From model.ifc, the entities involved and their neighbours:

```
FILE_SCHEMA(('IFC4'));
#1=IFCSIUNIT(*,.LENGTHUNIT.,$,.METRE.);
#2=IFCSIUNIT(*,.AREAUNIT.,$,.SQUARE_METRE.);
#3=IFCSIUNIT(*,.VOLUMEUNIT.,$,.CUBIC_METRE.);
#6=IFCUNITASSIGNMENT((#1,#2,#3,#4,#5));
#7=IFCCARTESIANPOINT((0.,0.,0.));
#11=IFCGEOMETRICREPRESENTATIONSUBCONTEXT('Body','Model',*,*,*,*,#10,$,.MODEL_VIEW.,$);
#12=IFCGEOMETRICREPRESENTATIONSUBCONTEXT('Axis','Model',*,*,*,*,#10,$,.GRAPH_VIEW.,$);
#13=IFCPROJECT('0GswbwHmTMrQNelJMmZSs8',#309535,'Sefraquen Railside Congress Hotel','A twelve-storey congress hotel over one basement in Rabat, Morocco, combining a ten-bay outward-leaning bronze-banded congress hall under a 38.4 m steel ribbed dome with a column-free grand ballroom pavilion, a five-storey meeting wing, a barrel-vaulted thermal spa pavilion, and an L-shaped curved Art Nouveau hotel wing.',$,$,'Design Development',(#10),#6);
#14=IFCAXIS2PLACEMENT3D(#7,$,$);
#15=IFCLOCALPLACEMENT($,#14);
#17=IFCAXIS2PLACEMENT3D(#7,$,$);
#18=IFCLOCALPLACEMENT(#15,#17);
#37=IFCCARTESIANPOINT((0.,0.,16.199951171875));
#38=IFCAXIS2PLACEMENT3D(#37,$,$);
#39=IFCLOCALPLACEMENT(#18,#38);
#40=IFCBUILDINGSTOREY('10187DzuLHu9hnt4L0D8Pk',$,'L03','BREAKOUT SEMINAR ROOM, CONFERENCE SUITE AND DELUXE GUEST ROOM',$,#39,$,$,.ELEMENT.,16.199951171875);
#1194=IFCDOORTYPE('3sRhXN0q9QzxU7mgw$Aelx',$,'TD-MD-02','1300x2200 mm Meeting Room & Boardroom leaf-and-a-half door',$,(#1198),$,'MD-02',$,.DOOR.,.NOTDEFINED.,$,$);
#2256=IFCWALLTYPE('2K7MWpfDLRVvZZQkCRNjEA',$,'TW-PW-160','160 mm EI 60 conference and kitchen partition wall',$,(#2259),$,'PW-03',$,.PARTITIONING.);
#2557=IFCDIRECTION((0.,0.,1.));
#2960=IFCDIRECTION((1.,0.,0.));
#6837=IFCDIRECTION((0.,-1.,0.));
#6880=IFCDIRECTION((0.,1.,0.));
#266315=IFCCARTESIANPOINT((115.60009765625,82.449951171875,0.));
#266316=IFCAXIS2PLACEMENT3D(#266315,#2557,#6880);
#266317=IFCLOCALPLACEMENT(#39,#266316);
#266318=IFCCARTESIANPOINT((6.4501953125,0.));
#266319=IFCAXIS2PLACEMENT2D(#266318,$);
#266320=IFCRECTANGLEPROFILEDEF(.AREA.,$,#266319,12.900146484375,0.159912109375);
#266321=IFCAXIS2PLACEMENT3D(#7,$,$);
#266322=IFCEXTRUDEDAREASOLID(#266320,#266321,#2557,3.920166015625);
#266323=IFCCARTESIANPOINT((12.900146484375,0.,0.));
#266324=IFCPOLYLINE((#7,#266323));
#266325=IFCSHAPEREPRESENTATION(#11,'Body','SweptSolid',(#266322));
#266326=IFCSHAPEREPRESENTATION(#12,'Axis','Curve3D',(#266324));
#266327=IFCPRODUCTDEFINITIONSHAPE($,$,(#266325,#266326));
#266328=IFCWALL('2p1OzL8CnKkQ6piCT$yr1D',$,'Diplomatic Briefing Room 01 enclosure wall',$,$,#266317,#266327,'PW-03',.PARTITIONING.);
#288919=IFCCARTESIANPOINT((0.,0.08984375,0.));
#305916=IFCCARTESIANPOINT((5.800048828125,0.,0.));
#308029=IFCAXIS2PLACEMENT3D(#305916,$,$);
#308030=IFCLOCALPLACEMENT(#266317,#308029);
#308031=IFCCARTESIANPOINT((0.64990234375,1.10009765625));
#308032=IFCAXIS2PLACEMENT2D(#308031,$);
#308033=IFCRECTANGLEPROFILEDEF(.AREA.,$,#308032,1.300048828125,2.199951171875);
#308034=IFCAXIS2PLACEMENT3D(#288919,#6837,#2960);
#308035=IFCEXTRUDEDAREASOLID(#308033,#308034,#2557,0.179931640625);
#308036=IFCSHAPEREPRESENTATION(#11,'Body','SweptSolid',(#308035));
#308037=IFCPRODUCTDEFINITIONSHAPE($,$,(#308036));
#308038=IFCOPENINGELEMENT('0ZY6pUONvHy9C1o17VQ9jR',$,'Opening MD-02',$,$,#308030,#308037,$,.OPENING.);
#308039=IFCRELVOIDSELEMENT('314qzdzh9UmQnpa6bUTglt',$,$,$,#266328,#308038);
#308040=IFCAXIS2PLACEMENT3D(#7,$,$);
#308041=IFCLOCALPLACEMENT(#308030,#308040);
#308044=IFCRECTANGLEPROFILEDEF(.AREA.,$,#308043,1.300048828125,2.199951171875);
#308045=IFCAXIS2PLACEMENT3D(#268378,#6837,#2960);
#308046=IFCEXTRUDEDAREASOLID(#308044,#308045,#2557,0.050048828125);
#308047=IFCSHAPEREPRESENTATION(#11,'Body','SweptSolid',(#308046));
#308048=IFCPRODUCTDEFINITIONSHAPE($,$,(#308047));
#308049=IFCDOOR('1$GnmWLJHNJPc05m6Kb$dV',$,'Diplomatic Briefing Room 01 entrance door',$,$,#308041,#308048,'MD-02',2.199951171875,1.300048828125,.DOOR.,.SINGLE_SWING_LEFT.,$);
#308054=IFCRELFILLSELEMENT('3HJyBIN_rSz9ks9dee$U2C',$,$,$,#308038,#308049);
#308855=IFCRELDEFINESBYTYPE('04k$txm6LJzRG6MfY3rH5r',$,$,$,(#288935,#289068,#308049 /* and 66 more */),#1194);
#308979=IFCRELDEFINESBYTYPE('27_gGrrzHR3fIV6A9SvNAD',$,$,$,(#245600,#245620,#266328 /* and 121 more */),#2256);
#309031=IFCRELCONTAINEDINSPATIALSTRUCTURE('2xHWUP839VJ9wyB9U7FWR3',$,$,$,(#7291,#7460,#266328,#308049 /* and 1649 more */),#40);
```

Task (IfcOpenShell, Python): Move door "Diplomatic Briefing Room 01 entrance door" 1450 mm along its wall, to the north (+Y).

```python
import ifcopenshell
import ifcopenshell.api.geometry
import ifcopenshell.util.placement
import ifcopenshell.util.unit

model = ifcopenshell.open("model.ifc")
unit_scale = ifcopenshell.util.unit.calculate_unit_scale(model)

door = model.by_id(308049)
opening = door.FillsVoids[0].RelatingOpeningElement
wall = opening.VoidsElements[0].RelatingBuildingElement

wall_matrix = ifcopenshell.util.placement.get_local_placement(wall.ObjectPlacement)
shift = wall_matrix[:3, 0] * 1.45 / unit_scale
before = ifcopenshell.util.placement.get_local_placement(door.ObjectPlacement)[:3, 3].copy()

# The door is placed relative to its opening, so it follows when the opening moves.
matrix = ifcopenshell.util.placement.get_local_placement(opening.ObjectPlacement)
matrix[:3, 3] += shift
ifcopenshell.api.geometry.edit_object_placement(
    model, product=opening, matrix=matrix, is_si=False, should_transform_children=True
)

after = ifcopenshell.util.placement.get_local_placement(door.ObjectPlacement)[:3, 3]
print("door moved by", (after - before).round(3) + 0.0)

model.write("model_edited.ifc")
```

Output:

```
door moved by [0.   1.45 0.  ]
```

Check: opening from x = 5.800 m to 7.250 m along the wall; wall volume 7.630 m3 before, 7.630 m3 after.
